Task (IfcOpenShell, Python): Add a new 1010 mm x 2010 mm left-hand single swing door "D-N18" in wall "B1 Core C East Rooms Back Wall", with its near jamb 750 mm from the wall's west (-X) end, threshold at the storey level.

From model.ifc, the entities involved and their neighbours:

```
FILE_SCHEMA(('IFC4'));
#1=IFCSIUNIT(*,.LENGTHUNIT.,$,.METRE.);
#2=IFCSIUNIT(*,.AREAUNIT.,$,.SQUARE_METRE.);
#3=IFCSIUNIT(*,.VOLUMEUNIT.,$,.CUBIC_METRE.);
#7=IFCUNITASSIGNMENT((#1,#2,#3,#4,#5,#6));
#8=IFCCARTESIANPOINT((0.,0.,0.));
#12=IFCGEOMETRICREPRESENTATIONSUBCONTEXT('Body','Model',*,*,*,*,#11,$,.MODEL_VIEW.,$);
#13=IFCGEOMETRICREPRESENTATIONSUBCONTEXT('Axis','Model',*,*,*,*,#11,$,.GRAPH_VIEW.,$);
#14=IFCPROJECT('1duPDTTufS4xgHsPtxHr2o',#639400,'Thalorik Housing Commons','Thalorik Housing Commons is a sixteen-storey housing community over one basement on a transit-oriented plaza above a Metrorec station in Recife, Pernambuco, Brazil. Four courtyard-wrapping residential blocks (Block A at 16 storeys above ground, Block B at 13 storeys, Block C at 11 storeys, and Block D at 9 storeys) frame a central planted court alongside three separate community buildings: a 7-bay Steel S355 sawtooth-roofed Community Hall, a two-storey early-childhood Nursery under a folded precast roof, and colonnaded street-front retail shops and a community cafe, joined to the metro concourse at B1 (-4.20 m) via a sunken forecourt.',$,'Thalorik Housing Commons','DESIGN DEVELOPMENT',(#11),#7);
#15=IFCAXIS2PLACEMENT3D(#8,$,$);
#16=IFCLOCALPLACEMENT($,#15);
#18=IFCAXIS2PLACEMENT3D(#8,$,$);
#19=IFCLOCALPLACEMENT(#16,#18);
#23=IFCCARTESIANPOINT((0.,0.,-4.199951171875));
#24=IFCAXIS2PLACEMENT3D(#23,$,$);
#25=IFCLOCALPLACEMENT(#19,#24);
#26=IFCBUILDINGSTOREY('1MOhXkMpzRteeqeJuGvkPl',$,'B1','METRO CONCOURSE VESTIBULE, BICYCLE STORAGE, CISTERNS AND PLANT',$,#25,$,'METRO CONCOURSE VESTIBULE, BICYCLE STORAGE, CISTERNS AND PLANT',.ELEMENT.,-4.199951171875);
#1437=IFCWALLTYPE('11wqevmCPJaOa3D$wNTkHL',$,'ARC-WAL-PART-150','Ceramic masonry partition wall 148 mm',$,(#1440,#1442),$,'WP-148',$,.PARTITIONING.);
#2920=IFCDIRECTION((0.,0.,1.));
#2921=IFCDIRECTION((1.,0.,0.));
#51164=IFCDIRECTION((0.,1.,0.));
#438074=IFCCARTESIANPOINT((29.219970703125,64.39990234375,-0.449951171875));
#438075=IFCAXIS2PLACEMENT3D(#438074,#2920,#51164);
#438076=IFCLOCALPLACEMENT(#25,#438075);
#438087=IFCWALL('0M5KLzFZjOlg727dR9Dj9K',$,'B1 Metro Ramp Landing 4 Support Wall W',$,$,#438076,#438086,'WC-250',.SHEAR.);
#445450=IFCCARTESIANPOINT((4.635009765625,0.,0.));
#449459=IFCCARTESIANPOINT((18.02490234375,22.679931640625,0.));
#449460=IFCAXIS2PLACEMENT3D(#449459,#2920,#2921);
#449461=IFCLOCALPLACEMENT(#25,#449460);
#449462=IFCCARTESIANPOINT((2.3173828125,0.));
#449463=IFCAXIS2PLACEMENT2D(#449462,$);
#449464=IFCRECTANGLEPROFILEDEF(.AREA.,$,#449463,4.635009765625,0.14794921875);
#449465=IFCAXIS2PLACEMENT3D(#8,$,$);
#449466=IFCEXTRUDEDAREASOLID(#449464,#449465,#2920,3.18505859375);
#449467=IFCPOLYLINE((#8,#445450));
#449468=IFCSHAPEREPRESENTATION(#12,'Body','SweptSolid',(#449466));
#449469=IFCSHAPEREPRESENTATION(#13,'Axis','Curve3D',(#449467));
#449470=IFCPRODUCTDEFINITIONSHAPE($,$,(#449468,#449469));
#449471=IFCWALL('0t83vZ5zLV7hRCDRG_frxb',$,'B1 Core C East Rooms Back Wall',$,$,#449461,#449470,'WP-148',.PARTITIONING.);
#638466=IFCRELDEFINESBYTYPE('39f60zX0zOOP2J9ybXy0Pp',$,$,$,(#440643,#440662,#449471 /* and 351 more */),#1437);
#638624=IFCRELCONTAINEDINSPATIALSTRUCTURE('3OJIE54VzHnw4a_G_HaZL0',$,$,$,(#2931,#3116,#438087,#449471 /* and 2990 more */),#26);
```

```python
import numpy as np
import ifcopenshell
import ifcopenshell.api.feature
import ifcopenshell.api.geometry
import ifcopenshell.api.root
import ifcopenshell.api.spatial
import ifcopenshell.geom
import ifcopenshell.util.element
import ifcopenshell.util.placement
import ifcopenshell.util.representation
import ifcopenshell.util.shape
import ifcopenshell.util.unit

model = ifcopenshell.open("model.ifc")
unit_scale = ifcopenshell.util.unit.calculate_unit_scale(model)
settings = ifcopenshell.geom.settings()


def volume(element):
    """Net volume in cubic metres, openings subtracted."""
    shape = ifcopenshell.geom.create_shape(settings, element)
    return ifcopenshell.util.shape.get_volume(shape.geometry)


wall = model.by_guid("0t83vZ5zLV7hRCDRG_frxb")
storey = ifcopenshell.util.element.get_container(wall, ifc_class="IfcBuildingStorey")
context = ifcopenshell.util.representation.get_context(model, "Model", "Body", "MODEL_VIEW")
before = volume(wall)

width, height, from_end, sill = 1.01, 2.01, 0.75, 0.0  # metres

# The wall runs along its own X axis, and the end named is its -X end.
wall_shape = ifcopenshell.geom.create_shape(settings, wall)
x, y, z = ifcopenshell.util.shape.get_vertices(wall_shape.geometry).T
start = x.min() + from_end
face, thickness = float(y.min()), float(y.max() - y.min())
wall_matrix = ifcopenshell.util.placement.get_local_placement(wall.ObjectPlacement)
level = ifcopenshell.util.placement.get_local_placement(storey.ObjectPlacement)[2, 3]


def in_wall(x, y):
    """Placement at x, y metres in the wall's axes, at sill height."""
    matrix = wall_matrix.copy()
    matrix[:, 3] = wall_matrix @ np.array([x / unit_scale, y / unit_scale, 0.0, 1.0])
    matrix[2, 3] = level + sill / unit_scale
    return matrix


# Opening: a box that overshoots both wall faces by 50 mm.
opening = ifcopenshell.api.root.create_entity(model, ifc_class="IfcOpeningElement", predefined_type="OPENING")
box = ifcopenshell.api.geometry.add_wall_representation(
    model, context=context, length=width, height=height, thickness=thickness + 0.1
)
ifcopenshell.api.geometry.assign_representation(model, product=opening, representation=box)
ifcopenshell.api.geometry.edit_object_placement(model, product=opening, matrix=in_wall(start, face - 0.05), is_si=False)
ifcopenshell.api.feature.add_feature(model, feature=opening, element=wall)

door = ifcopenshell.api.root.create_entity(model, ifc_class="IfcDoor", name="D-N18", predefined_type="DOOR")
door.OverallWidth, door.OverallHeight = width / unit_scale, height / unit_scale
door.OperationType = "SINGLE_SWING_LEFT"
body = ifcopenshell.api.geometry.add_door_representation(
    model,
    context=context,
    overall_width=door.OverallWidth,
    overall_height=door.OverallHeight,
    operation_type="SINGLE_SWING_LEFT",
    lining_properties={"LiningDepth": thickness / unit_scale, "ThresholdDepth": thickness / unit_scale},
)
ifcopenshell.api.geometry.assign_representation(model, product=door, representation=body)
ifcopenshell.api.spatial.assign_container(model, products=[door], relating_structure=storey)
ifcopenshell.api.feature.add_filling(model, opening=opening, element=door)

# The lining spans the wall, so the door starts at the wall face.
ifcopenshell.api.geometry.edit_object_placement(model, product=door, matrix=in_wall(start, face), is_si=False)

after = volume(wall)

print(f"wall volume {before:.3f} -> {after:.3f} m3")

model.write("model_edited.ifc")
```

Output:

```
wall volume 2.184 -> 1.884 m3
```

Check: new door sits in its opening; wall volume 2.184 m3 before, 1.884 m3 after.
